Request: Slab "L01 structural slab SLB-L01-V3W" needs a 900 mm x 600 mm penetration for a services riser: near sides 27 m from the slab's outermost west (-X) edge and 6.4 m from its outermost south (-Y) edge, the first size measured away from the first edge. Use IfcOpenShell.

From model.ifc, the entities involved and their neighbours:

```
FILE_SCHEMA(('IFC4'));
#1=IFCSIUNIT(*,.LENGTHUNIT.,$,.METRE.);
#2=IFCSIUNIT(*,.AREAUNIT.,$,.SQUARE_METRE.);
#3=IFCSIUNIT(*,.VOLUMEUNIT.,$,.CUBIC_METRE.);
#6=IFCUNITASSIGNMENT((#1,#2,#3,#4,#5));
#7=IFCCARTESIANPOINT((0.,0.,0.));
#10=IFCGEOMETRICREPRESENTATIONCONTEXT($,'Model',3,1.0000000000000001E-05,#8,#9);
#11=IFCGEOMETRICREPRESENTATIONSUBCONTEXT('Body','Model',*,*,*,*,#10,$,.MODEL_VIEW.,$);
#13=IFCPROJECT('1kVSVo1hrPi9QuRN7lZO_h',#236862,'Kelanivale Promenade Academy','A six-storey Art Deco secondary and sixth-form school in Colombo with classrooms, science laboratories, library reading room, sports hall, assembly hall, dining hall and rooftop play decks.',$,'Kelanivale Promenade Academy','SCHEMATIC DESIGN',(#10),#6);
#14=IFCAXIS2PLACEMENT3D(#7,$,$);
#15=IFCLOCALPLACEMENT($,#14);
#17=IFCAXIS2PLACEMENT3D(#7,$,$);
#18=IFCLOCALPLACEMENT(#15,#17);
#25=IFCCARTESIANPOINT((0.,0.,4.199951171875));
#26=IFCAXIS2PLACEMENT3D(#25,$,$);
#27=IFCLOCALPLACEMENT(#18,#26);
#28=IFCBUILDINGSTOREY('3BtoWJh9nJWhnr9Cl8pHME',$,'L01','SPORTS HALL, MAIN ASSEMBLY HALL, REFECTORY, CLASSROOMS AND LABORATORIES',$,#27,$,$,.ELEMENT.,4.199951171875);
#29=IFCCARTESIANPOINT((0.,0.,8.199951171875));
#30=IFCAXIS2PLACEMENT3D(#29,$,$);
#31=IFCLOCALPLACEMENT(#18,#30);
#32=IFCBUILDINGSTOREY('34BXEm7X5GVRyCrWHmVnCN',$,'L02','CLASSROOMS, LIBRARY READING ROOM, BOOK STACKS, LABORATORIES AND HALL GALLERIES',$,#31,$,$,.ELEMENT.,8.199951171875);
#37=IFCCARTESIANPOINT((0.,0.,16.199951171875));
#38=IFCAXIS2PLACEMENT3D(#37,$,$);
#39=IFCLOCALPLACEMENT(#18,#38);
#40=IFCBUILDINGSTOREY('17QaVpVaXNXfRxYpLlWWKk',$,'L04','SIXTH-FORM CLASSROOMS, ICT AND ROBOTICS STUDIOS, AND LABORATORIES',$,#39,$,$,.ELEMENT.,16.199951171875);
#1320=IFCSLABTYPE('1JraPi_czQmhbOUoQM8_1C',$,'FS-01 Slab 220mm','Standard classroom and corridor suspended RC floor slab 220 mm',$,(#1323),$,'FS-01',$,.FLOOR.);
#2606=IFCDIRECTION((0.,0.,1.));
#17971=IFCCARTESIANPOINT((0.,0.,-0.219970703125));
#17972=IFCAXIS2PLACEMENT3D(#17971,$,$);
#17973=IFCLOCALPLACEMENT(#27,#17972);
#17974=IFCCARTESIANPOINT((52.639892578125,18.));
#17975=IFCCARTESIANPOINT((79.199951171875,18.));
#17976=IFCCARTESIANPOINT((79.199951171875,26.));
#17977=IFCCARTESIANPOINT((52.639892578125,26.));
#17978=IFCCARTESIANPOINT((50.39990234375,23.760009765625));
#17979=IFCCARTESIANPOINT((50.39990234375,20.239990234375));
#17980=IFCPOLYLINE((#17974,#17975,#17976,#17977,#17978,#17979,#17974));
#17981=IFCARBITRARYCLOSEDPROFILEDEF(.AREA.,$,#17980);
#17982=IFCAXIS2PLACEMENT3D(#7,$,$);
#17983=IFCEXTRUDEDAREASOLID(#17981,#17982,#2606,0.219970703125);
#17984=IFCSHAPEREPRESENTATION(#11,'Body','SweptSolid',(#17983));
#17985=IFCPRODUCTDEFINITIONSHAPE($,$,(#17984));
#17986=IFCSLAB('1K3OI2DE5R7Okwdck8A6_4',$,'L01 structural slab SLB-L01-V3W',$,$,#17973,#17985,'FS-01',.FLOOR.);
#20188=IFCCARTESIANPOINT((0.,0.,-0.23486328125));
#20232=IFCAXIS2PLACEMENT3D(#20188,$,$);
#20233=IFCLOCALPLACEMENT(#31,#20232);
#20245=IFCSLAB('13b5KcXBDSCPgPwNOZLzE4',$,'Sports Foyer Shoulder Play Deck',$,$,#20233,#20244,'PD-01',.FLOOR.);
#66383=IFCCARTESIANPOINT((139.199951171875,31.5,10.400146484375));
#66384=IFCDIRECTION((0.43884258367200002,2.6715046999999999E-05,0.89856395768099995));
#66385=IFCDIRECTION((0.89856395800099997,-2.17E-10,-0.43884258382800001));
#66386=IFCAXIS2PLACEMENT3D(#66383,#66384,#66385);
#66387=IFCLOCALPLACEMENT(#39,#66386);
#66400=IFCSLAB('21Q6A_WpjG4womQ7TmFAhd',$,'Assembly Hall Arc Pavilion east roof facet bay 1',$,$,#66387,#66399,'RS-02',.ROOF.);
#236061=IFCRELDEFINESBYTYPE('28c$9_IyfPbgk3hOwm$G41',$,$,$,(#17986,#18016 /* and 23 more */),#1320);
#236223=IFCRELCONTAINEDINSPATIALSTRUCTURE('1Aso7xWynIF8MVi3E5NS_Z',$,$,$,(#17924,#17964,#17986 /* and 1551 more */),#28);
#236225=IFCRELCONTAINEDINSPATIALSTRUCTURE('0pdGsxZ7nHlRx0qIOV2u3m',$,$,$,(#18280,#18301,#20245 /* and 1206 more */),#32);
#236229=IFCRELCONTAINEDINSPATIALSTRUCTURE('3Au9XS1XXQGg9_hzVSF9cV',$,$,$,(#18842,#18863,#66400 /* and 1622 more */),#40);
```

```python
import numpy as np
import ifcopenshell
import ifcopenshell.api.feature
import ifcopenshell.api.geometry
import ifcopenshell.api.root
import ifcopenshell.geom
import ifcopenshell.util.placement
import ifcopenshell.util.representation
import ifcopenshell.util.shape
import ifcopenshell.util.unit

model = ifcopenshell.open("model.ifc")
unit_scale = ifcopenshell.util.unit.calculate_unit_scale(model)
settings = ifcopenshell.geom.settings()


def volume(element):
    """Net volume in cubic metres, openings subtracted."""
    shape = ifcopenshell.geom.create_shape(settings, element)
    return ifcopenshell.util.shape.get_volume(shape.geometry)


slab = model.by_guid("1K3OI2DE5R7Okwdck8A6_4")
before = volume(slab)

# Extent in the slab's own axes, in metres. The edges named are its -X and -Y sides.
slab_shape = ifcopenshell.geom.create_shape(settings, slab)
vertices = ifcopenshell.util.shape.get_vertices(slab_shape.geometry)
x_min, y_min, bottom = vertices.min(axis=0)
top = vertices[:, 2].max()

opening = ifcopenshell.api.root.create_entity(model, ifc_class="IfcOpeningElement", name="Services riser opening", predefined_type="OPENING")
context = ifcopenshell.util.representation.get_context(model, "Model", "Body", "MODEL_VIEW")
width, depth = 0.9, 0.6
outline = [(0.0, 0.0), (width, 0.0), (width, depth), (0.0, depth), (0.0, 0.0)]
# Overshoot both faces by 50 mm so the cut is clean.
shape = ifcopenshell.api.geometry.add_slab_representation(
    model, context=context, depth=top - bottom + 0.1, polyline=outline
)
ifcopenshell.api.geometry.assign_representation(model, product=opening, representation=shape)

matrix = ifcopenshell.util.placement.get_local_placement(slab.ObjectPlacement)
matrix[:, 3] = matrix @ np.append(np.array([x_min + 27, y_min + 6.4, bottom - 0.05]) / unit_scale, 1.0)
ifcopenshell.api.geometry.edit_object_placement(model, product=opening, matrix=matrix, is_si=False)
ifcopenshell.api.feature.add_feature(model, feature=opening, element=slab)

after = volume(slab)

print(f"slab volume {before:.3f} -> {after:.3f} m3")

model.write("model_updated.ifc")
```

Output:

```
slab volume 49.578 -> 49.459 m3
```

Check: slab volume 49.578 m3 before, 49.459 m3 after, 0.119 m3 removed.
